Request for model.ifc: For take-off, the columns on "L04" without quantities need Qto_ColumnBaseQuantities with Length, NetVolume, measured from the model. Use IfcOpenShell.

First a look at what the model holds.

```python
import ifcopenshell
import ifcopenshell.util.element
import ifcopenshell.util.unit

model = ifcopenshell.open("model.ifc")
print(model.schema)
for unit_type in ("LENGTHUNIT", "AREAUNIT", "VOLUMEUNIT"):
    print(unit_type, ifcopenshell.util.unit.calculate_unit_scale(model, unit_type))
storey = next(s for s in model.by_type("IfcBuildingStorey") if s.Name == "L04")
columns = [e for e in ifcopenshell.util.element.get_decomposition(storey) if e.is_a("IfcColumn")]
for e in sorted(columns, key=lambda e: e.id()):
    print(e.id(), e.is_a(), e.Name, list(ifcopenshell.util.element.get_psets(e, qtos_only=True)), sep=" | ")
```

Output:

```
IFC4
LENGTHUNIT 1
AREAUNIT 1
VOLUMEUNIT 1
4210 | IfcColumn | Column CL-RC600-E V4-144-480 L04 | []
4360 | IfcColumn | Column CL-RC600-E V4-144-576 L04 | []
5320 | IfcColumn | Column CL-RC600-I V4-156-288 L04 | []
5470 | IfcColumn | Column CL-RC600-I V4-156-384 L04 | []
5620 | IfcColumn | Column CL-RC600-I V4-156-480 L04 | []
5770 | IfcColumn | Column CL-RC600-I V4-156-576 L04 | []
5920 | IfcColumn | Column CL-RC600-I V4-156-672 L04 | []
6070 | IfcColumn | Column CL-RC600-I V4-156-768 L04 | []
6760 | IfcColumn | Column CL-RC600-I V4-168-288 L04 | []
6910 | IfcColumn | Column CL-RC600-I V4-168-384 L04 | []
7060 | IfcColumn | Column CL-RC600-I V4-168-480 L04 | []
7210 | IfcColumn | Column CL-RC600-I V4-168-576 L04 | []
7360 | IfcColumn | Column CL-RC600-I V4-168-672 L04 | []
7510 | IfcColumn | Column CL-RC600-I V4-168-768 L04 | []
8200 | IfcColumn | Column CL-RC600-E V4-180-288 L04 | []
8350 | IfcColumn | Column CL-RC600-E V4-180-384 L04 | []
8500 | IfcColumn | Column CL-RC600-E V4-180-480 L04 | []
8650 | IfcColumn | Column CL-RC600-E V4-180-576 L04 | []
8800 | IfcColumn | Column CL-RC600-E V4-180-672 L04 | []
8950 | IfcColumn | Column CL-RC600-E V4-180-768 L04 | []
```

```python
import ifcopenshell
import ifcopenshell.api.pset
import ifcopenshell.geom
import ifcopenshell.util.element
import ifcopenshell.util.shape
import ifcopenshell.util.unit

model = ifcopenshell.open("model.ifc")
unit_scale = ifcopenshell.util.unit.calculate_unit_scale(model)
volume_scale = ifcopenshell.util.unit.calculate_unit_scale(model, "VOLUMEUNIT")
settings = ifcopenshell.geom.settings()

storey = next(s for s in model.by_type("IfcBuildingStorey") if s.Name == "L04")
columns = [e for e in ifcopenshell.util.element.get_decomposition(storey) if e.is_a("IfcColumn")]

for e in sorted(columns, key=lambda e: e.id()):
    if ifcopenshell.util.element.get_psets(e, qtos_only=True, should_inherit=False):
        continue
    # Geometry comes back in metres, in the element's own axes.
    shape = ifcopenshell.geom.create_shape(settings, e)
    values = {
        "Length": ifcopenshell.util.shape.get_z(shape.geometry) / unit_scale,
        "NetVolume": ifcopenshell.util.shape.get_volume(shape.geometry) / volume_scale,
    }
    qto = ifcopenshell.api.pset.add_qto(model, product=e, name="Qto_ColumnBaseQuantities")
    ifcopenshell.api.pset.edit_qto(model, qto=qto, properties=values)
    print(e.id(), {k: round(v, 3) for k, v in values.items()})

model.write("model_edited.ifc")
```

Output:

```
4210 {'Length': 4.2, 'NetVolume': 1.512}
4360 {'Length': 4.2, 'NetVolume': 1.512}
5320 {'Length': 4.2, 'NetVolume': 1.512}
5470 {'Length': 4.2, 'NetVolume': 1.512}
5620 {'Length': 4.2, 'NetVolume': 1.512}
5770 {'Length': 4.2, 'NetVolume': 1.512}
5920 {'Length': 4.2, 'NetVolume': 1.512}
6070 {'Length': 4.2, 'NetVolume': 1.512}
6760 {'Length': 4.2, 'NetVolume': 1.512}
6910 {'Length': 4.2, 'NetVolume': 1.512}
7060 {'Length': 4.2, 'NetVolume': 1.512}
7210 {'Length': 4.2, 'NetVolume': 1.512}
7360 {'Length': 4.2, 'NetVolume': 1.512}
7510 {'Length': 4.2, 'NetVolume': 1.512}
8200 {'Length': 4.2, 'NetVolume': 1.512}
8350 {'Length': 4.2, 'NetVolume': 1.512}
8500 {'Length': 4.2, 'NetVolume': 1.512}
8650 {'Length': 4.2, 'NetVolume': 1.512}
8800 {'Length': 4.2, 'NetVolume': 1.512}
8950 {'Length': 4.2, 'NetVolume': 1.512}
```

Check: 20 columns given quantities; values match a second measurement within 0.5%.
